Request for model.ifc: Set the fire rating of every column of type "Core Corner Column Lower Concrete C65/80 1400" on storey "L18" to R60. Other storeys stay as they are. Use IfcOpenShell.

First a look at what the model holds.

```python
import ifcopenshell
import ifcopenshell.util.element

model = ifcopenshell.open("model.ifc")
print(model.schema)
storey = next(s for s in model.by_type("IfcBuildingStorey") if s.Name == "L18")
columns = [e for e in ifcopenshell.util.element.get_decomposition(storey) if e.is_a("IfcColumn")]
seen = {}
for e in columns:
    element_type = ifcopenshell.util.element.get_type(e)
    key = (element_type.Name if element_type != e and element_type else None, ifcopenshell.util.element.get_pset(e, "Pset_ColumnCommon", "FireRating"))
    seen[key] = seen.get(key, 0) + 1
for (name, value), count in sorted(seen.items(), key=str):
    print(count, "x", name, "|", value)
```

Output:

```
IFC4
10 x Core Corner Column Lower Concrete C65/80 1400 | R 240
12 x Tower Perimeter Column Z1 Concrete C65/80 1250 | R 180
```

```python
import ifcopenshell
import ifcopenshell.api.pset
import ifcopenshell.util.element

model = ifcopenshell.open("model.ifc")

storey = next(s for s in model.by_type("IfcBuildingStorey") if s.Name == "L18")
columns = [e for e in ifcopenshell.util.element.get_decomposition(storey) if e.is_a("IfcColumn")]

count = 0
for e in columns:
    element_type = ifcopenshell.util.element.get_type(e)
    if element_type in (None, e) or element_type.Name != "Core Corner Column Lower Concrete C65/80 1400":
        continue
    found = ifcopenshell.util.element.get_pset(e, "Pset_ColumnCommon", should_inherit=False)
    if found:
        pset = model.by_id(found["id"])
        if len(ifcopenshell.util.element.get_elements_by_pset(pset)) > 1:
            pset = ifcopenshell.api.pset.unshare_pset(model, products=[e], pset=pset)[0]
    else:
        pset = ifcopenshell.api.pset.add_pset(model, product=e, name="Pset_ColumnCommon")
    ifcopenshell.api.pset.edit_pset(model, pset=pset, properties={"FireRating": "R60"})
    count += 1

print(count, "columns updated")

model.write("model_rev.ifc")
```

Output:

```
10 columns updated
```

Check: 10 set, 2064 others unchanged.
